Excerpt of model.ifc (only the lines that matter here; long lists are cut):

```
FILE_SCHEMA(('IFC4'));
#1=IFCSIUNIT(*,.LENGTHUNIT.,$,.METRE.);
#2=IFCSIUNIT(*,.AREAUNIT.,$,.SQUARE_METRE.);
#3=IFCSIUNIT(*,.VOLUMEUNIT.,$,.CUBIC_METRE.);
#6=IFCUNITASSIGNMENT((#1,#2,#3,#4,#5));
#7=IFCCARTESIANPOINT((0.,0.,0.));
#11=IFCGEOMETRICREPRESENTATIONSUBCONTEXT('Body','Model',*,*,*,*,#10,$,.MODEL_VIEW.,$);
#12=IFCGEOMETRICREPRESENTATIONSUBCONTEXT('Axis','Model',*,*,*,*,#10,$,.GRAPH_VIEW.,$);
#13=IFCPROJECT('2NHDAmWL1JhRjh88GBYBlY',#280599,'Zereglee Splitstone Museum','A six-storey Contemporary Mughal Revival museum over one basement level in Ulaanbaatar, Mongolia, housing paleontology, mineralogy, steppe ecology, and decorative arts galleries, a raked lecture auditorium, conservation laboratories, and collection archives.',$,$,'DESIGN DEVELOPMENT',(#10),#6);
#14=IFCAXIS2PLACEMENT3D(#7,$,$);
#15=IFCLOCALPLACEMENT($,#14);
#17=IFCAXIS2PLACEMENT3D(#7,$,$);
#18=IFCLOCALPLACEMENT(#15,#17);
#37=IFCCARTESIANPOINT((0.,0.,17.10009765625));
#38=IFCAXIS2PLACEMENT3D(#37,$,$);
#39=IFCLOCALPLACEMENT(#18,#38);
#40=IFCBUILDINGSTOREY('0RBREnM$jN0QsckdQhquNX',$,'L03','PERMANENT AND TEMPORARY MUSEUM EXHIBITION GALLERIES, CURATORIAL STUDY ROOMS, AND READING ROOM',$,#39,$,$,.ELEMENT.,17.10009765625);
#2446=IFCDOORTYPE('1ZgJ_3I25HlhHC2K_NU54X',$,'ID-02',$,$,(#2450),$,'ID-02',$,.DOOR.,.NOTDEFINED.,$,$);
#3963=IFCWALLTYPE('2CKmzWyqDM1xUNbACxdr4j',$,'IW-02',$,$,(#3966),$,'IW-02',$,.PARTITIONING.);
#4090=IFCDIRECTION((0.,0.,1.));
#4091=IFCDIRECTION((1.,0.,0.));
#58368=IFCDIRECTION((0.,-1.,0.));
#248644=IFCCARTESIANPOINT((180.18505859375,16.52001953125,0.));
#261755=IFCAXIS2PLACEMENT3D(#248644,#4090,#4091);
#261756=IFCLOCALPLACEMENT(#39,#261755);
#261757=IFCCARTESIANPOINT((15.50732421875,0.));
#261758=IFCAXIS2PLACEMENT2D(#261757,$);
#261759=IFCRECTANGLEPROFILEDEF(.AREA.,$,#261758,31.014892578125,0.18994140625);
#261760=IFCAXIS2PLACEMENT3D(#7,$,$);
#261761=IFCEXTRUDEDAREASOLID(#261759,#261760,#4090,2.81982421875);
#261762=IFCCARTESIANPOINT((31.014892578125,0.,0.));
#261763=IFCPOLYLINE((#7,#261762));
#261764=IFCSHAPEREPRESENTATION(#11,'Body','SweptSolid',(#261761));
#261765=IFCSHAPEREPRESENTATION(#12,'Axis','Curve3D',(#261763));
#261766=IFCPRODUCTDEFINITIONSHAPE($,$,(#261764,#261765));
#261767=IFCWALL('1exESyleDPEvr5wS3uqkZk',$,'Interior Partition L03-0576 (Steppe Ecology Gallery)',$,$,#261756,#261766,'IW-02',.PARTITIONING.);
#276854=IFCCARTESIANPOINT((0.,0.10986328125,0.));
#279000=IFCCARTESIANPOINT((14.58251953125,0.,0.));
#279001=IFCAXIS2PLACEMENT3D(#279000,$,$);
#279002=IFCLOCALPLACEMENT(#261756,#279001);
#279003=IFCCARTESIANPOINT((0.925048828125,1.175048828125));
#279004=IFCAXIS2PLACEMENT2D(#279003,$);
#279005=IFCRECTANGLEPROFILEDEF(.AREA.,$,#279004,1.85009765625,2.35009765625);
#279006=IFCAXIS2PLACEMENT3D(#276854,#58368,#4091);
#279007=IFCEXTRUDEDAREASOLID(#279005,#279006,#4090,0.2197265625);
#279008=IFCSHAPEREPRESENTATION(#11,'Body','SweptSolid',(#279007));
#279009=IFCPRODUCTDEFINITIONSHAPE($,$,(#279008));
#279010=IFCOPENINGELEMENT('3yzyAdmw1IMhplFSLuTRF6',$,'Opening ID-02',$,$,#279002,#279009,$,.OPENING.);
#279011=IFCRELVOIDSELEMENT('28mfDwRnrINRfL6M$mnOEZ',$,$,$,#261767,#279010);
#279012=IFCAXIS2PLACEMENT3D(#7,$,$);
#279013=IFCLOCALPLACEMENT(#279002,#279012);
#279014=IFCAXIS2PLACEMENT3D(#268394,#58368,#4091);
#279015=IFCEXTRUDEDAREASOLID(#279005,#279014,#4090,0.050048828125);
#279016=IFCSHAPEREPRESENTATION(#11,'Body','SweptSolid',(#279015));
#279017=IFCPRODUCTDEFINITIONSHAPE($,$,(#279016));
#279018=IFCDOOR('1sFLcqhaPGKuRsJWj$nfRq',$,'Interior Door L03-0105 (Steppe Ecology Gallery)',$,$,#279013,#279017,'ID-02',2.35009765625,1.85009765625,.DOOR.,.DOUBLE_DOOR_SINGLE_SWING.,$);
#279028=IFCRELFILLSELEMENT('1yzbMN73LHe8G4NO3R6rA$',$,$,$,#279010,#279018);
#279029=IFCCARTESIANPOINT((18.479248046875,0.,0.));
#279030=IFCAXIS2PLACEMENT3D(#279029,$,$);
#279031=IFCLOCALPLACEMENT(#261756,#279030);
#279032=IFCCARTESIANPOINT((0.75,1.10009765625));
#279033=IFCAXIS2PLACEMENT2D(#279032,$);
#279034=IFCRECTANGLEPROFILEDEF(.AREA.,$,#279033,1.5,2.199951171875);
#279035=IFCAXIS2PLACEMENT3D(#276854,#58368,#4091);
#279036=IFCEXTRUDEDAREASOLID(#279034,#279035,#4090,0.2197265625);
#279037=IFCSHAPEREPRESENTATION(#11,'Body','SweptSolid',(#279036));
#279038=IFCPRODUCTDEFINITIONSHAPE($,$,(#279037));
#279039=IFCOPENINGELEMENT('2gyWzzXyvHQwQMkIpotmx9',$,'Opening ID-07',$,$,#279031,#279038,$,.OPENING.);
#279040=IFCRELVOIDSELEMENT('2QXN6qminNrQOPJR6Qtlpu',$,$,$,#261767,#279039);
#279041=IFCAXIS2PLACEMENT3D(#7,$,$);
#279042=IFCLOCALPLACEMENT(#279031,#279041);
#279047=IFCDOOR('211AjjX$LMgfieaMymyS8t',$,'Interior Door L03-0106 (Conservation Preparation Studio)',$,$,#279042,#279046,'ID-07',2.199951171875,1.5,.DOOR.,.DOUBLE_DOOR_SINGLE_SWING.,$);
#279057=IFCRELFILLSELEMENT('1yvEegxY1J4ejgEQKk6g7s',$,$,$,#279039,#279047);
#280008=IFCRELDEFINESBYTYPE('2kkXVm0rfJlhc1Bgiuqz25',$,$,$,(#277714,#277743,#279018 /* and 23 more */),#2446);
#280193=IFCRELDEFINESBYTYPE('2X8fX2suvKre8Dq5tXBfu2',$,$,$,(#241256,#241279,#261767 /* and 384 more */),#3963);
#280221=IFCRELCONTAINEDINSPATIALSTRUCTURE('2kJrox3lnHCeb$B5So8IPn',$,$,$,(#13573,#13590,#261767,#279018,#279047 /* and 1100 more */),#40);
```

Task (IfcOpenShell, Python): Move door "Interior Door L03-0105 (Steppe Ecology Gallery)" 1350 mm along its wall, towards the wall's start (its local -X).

```python
import ifcopenshell
import ifcopenshell.api.geometry
import ifcopenshell.util.placement

model = ifcopenshell.open("model.ifc")

door = model.by_guid("1sFLcqhaPGKuRsJWj$nfRq")
opening = door.FillsVoids[0].RelatingOpeningElement
wall = opening.VoidsElements[0].RelatingBuildingElement

wall_matrix = ifcopenshell.util.placement.get_local_placement(wall.ObjectPlacement)
shift = wall_matrix[:3, 0] * -1.35
before = ifcopenshell.util.placement.get_local_placement(door.ObjectPlacement)[:3, 3].copy()

# The door is placed relative to its opening, so it follows when the opening moves.
matrix = ifcopenshell.util.placement.get_local_placement(opening.ObjectPlacement)
matrix[:3, 3] += shift
ifcopenshell.api.geometry.edit_object_placement(
    model, product=opening, matrix=matrix, is_si=False, should_transform_children=True
)

after = ifcopenshell.util.placement.get_local_placement(door.ObjectPlacement)[:3, 3]
print("door moved by", (after - before).round(3) + 0.0)

model.write("model-out.ifc")
```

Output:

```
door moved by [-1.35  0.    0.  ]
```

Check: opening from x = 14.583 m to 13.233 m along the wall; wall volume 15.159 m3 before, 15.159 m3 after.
